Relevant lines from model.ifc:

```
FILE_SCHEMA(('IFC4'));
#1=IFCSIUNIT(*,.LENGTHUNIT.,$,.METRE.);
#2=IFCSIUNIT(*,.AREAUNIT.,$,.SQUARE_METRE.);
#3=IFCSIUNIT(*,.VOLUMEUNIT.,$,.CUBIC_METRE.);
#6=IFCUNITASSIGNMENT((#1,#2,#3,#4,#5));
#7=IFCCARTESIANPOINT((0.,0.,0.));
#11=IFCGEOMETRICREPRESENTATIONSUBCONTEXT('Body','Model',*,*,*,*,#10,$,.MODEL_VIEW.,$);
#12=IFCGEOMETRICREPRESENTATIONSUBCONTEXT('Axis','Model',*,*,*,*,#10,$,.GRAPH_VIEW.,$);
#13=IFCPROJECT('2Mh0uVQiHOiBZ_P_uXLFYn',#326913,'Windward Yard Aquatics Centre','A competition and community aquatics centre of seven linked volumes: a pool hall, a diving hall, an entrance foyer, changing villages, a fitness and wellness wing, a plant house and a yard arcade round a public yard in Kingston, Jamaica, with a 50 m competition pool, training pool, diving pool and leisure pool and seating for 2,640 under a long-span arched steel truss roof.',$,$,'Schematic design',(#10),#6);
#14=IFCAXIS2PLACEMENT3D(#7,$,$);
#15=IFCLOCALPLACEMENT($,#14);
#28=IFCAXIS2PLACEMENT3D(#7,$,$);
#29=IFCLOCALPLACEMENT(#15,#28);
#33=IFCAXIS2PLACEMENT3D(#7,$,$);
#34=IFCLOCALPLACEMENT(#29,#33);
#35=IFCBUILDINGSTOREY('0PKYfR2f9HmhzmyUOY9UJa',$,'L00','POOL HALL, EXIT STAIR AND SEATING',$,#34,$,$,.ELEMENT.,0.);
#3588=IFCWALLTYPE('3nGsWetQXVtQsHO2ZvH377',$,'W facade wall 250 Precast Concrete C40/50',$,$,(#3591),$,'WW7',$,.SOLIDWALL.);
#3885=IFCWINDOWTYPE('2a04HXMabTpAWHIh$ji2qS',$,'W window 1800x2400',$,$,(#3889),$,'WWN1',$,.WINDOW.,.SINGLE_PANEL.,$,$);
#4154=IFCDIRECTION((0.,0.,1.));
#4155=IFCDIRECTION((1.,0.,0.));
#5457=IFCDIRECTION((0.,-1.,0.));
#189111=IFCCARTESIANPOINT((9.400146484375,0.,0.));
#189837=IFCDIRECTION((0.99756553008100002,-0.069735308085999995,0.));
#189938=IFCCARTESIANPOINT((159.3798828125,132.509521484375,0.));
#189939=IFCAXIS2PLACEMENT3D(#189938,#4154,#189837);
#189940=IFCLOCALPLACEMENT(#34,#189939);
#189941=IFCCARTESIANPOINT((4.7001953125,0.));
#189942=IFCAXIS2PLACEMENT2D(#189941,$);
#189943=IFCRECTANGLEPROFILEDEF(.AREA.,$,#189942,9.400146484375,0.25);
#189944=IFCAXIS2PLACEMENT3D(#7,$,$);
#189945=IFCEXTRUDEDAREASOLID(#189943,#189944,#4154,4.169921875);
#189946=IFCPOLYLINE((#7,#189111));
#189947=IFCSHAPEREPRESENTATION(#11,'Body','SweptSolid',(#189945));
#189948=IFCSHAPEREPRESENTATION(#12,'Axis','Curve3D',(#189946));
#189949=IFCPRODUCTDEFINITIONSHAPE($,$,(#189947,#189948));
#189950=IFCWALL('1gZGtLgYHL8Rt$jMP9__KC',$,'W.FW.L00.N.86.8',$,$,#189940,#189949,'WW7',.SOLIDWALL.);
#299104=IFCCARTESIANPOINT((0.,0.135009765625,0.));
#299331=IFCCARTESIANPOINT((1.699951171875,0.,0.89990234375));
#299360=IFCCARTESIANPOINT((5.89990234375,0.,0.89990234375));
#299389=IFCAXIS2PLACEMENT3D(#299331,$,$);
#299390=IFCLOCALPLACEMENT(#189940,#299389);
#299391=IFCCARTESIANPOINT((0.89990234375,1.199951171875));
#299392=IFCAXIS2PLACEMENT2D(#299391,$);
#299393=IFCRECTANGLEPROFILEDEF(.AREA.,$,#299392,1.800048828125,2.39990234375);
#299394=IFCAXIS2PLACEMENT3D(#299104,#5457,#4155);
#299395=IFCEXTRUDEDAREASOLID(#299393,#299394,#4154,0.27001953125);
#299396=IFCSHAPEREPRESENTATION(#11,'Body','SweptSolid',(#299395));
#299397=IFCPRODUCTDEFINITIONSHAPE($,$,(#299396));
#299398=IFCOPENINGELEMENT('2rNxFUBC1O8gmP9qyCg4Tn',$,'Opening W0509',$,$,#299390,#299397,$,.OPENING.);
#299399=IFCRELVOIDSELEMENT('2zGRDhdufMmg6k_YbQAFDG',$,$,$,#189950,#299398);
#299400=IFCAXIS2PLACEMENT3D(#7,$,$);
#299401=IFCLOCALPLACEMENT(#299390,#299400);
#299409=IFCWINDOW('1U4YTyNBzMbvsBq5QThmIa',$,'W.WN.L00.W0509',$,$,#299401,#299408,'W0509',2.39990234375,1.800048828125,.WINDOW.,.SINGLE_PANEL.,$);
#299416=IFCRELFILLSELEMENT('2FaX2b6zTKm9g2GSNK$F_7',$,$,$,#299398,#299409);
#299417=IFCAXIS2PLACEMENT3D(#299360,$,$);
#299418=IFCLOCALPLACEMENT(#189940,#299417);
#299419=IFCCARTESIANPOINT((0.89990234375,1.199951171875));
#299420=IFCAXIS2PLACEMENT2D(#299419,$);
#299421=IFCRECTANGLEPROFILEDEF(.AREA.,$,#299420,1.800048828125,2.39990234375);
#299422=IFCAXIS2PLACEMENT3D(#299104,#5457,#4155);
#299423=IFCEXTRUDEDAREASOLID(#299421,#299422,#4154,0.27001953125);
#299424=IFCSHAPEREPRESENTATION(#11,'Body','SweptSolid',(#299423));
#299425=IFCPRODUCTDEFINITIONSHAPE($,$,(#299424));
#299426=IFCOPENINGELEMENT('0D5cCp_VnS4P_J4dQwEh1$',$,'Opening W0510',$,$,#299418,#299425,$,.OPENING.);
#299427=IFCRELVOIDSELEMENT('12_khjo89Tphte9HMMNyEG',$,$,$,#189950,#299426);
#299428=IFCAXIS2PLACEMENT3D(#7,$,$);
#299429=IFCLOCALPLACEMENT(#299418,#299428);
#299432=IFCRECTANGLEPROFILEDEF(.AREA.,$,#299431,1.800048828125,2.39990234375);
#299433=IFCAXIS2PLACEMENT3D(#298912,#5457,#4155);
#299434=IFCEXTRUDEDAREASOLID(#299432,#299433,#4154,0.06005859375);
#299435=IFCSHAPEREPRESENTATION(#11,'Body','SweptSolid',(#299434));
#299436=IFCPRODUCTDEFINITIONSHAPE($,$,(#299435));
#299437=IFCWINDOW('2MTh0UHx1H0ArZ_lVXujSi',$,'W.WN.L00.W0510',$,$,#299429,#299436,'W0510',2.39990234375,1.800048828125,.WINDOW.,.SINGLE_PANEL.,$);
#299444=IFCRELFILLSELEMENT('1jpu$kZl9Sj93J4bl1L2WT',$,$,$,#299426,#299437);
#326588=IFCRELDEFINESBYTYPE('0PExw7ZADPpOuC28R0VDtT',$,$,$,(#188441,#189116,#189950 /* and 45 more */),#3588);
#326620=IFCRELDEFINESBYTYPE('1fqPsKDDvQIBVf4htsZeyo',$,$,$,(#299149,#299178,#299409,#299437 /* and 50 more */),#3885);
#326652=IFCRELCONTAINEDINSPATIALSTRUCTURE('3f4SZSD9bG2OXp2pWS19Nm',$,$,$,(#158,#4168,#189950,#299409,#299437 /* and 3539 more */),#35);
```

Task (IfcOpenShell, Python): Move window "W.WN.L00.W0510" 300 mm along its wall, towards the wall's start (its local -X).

```python
import ifcopenshell
import ifcopenshell.api.geometry
import ifcopenshell.util.placement

model = ifcopenshell.open("model.ifc")

window = model.by_guid("2MTh0UHx1H0ArZ_lVXujSi")
opening = window.FillsVoids[0].RelatingOpeningElement
wall = opening.VoidsElements[0].RelatingBuildingElement

wall_matrix = ifcopenshell.util.placement.get_local_placement(wall.ObjectPlacement)
shift = wall_matrix[:3, 0] * -0.3
before = ifcopenshell.util.placement.get_local_placement(window.ObjectPlacement)[:3, 3].copy()

# The window is placed relative to its opening, so it follows when the opening moves.
matrix = ifcopenshell.util.placement.get_local_placement(opening.ObjectPlacement)
matrix[:3, 3] += shift
ifcopenshell.api.geometry.edit_object_placement(
    model, product=opening, matrix=matrix, is_si=False, should_transform_children=True
)

after = ifcopenshell.util.placement.get_local_placement(window.ObjectPlacement)[:3, 3]
print("window moved by", (after - before).round(3) + 0.0)

model.write("model_edited.ifc")
```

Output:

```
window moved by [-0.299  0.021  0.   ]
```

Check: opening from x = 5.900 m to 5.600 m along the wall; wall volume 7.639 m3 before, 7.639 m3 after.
